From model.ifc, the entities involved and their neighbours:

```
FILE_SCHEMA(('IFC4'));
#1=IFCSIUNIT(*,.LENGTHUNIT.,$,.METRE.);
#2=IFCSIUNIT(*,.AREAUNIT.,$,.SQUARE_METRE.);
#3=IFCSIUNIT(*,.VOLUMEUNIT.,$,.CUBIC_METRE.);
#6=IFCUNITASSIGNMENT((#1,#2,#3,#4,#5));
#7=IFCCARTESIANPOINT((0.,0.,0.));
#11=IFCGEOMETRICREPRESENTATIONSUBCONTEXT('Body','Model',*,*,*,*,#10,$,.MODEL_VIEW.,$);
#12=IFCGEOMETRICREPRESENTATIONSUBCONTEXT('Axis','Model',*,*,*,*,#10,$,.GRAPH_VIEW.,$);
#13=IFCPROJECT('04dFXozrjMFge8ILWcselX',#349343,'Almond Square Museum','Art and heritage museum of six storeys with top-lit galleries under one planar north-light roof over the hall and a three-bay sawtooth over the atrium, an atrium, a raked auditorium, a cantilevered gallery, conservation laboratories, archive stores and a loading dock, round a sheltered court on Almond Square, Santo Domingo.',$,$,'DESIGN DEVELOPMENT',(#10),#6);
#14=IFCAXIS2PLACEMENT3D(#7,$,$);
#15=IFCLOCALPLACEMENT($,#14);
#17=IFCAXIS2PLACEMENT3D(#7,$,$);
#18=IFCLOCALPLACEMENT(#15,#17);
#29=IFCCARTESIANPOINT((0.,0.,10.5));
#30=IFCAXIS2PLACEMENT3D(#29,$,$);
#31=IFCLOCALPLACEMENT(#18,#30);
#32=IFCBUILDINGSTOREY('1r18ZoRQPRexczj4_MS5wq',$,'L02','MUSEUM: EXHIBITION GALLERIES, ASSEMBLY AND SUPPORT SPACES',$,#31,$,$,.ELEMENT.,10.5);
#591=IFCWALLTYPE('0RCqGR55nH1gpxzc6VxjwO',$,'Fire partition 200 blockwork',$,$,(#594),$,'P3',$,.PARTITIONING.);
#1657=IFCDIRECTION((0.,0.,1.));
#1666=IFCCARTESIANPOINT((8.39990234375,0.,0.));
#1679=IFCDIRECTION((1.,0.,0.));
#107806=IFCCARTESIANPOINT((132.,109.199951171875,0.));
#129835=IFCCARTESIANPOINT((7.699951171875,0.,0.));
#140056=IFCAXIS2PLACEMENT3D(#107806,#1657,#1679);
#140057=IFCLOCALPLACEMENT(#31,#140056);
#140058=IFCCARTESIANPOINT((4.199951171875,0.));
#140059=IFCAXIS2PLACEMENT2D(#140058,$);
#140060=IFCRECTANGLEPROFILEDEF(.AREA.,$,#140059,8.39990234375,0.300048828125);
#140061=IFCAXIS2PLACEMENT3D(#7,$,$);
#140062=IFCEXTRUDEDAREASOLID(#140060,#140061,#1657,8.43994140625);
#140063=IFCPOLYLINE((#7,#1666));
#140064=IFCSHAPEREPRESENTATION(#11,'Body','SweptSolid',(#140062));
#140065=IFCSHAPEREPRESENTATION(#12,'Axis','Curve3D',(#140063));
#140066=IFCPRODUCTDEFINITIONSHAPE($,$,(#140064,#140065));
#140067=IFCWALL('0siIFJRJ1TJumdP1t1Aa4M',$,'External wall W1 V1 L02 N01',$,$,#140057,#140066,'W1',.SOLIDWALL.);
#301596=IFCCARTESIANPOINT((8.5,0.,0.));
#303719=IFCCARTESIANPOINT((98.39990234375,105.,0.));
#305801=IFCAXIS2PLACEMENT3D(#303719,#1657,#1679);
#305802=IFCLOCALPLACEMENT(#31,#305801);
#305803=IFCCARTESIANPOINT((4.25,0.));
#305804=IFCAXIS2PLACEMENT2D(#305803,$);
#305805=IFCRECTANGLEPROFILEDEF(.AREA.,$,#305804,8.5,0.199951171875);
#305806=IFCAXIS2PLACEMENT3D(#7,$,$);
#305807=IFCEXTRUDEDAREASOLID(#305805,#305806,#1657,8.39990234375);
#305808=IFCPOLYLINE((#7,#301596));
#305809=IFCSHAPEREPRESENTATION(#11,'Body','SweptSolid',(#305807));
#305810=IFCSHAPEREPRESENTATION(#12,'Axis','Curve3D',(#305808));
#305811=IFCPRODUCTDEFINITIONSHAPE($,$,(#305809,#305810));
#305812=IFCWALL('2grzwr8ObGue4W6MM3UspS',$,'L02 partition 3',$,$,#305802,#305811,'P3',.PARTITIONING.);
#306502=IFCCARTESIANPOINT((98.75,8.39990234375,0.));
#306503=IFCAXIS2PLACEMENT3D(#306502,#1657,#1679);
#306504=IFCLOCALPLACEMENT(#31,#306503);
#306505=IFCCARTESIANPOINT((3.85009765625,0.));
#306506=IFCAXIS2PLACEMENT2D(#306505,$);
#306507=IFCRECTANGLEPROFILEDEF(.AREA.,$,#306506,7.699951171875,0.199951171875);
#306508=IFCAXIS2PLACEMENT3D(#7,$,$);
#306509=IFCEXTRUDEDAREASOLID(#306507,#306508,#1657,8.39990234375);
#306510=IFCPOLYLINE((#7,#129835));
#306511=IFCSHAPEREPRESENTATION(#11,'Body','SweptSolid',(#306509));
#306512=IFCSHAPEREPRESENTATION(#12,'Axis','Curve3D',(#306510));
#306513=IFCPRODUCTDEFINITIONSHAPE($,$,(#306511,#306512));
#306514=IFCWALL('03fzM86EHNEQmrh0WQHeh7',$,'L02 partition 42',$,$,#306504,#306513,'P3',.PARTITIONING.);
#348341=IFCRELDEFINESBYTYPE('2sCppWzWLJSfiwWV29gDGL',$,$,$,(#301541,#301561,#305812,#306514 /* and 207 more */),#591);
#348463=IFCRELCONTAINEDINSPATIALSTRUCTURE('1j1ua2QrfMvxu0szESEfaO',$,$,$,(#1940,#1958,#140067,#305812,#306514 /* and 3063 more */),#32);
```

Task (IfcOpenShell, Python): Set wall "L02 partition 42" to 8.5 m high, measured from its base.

```python
import ifcopenshell
import ifcopenshell.geom
import ifcopenshell.util.representation
import ifcopenshell.util.shape
import ifcopenshell.util.unit

model = ifcopenshell.open("model.ifc")
unit_scale = ifcopenshell.util.unit.calculate_unit_scale(model)
settings = ifcopenshell.geom.settings()


def volume(element):
    """Net volume in cubic metres, openings subtracted."""
    shape = ifcopenshell.geom.create_shape(settings, element)
    return ifcopenshell.util.shape.get_volume(shape.geometry)


wall = model.by_id(306514)
before = volume(wall)

body = ifcopenshell.util.representation.get_representation(wall, "Model", "Body")
solid = body.Items[0]
old_height = solid.Depth
solid.Depth = 8.5 / unit_scale
after = volume(wall)

print(f"height {old_height:g} -> {solid.Depth:g}, volume {before:.3f} -> {after:.3f} m3")

model.write("model_v2.ifc")
```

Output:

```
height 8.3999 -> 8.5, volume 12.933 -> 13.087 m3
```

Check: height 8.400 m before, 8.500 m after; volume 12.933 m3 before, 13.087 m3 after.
